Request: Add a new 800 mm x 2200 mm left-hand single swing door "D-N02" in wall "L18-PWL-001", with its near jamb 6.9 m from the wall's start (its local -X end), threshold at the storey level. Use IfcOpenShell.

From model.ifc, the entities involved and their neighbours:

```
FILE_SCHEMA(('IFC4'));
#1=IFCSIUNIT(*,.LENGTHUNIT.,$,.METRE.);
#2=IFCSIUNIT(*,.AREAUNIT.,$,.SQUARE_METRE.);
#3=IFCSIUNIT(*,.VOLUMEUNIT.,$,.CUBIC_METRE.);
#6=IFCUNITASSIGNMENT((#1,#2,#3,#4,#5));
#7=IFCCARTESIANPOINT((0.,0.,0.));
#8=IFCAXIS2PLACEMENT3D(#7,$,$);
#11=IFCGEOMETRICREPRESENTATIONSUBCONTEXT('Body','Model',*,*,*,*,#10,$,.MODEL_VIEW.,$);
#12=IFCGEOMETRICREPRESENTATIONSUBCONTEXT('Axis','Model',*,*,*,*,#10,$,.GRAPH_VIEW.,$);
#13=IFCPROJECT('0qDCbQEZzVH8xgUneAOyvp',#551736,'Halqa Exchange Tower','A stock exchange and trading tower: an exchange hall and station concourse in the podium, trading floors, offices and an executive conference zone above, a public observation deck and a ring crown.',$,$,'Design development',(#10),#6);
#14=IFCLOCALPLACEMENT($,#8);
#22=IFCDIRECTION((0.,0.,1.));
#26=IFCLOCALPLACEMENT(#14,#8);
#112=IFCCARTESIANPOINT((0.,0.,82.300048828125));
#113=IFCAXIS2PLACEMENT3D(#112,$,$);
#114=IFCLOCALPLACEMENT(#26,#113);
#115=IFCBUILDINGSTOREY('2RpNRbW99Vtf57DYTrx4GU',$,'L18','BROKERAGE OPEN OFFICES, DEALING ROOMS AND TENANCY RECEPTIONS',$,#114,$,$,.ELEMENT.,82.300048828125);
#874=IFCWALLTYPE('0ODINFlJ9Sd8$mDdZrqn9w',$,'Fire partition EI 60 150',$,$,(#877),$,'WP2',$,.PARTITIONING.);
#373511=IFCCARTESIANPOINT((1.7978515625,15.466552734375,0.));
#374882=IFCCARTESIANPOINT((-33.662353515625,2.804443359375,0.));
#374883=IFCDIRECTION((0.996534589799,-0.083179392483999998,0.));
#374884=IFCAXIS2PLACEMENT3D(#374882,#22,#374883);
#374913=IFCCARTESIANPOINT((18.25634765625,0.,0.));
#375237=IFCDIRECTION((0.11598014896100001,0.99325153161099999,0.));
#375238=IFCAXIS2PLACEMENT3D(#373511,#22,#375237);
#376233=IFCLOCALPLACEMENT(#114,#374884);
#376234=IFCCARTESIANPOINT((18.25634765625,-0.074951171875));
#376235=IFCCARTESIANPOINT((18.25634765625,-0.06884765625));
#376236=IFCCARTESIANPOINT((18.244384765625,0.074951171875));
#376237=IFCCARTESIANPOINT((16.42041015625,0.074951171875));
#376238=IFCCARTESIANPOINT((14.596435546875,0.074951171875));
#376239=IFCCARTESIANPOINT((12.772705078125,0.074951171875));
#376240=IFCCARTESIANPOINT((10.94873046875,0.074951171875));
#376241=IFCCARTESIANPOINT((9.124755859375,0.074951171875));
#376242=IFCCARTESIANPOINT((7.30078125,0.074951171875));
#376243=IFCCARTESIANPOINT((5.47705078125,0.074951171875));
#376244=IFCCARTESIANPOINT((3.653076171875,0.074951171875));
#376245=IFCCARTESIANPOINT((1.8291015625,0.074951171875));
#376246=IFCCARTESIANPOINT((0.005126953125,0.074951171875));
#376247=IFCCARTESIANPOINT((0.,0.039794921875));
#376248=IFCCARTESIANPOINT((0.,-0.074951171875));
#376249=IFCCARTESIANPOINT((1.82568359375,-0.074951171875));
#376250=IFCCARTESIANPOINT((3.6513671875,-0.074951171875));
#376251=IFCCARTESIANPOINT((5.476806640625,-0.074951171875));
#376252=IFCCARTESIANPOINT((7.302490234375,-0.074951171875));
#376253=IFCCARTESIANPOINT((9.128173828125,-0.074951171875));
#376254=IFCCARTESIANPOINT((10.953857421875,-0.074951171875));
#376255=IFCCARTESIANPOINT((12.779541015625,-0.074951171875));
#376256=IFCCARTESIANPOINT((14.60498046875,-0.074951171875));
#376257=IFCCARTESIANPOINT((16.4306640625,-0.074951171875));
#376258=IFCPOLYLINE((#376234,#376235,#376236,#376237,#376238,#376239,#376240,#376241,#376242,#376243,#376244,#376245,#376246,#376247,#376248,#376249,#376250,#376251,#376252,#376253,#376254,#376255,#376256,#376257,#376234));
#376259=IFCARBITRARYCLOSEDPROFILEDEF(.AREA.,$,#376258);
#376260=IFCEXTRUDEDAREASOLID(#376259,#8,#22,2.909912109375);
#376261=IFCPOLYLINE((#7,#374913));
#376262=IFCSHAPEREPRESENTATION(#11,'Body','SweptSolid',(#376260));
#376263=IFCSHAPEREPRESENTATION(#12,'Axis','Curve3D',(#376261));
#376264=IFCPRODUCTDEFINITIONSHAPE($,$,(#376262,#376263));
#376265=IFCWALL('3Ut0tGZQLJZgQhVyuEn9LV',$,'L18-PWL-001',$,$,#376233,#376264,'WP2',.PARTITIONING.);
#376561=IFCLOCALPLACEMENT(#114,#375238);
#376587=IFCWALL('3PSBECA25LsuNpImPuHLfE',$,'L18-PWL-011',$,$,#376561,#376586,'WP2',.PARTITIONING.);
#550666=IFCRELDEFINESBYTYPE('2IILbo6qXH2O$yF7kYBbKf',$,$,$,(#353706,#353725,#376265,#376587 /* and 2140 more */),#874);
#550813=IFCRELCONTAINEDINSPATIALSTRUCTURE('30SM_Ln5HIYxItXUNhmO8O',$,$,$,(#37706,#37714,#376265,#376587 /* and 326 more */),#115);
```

```python
import numpy as np
import ifcopenshell
import ifcopenshell.api.feature
import ifcopenshell.api.geometry
import ifcopenshell.api.root
import ifcopenshell.api.spatial
import ifcopenshell.geom
import ifcopenshell.util.element
import ifcopenshell.util.placement
import ifcopenshell.util.representation
import ifcopenshell.util.shape
import ifcopenshell.util.unit

model = ifcopenshell.open("model.ifc")
unit_scale = ifcopenshell.util.unit.calculate_unit_scale(model)
settings = ifcopenshell.geom.settings()


def volume(element):
    """Net volume in cubic metres, openings subtracted."""
    shape = ifcopenshell.geom.create_shape(settings, element)
    return ifcopenshell.util.shape.get_volume(shape.geometry)


wall = model.by_guid("3Ut0tGZQLJZgQhVyuEn9LV")
storey = ifcopenshell.util.element.get_container(wall, ifc_class="IfcBuildingStorey")
context = ifcopenshell.util.representation.get_context(model, "Model", "Body", "MODEL_VIEW")
before = volume(wall)

width, height, from_end, sill = 0.8, 2.2, 6.9, 0.0  # metres

# The wall runs along its own X axis, and the end named is its -X end.
wall_shape = ifcopenshell.geom.create_shape(settings, wall)
x, y, z = ifcopenshell.util.shape.get_vertices(wall_shape.geometry).T
start = x.min() + from_end
face, thickness = float(y.min()), float(y.max() - y.min())
wall_matrix = ifcopenshell.util.placement.get_local_placement(wall.ObjectPlacement)
level = ifcopenshell.util.placement.get_local_placement(storey.ObjectPlacement)[2, 3]


def in_wall(x, y):
    """Placement at x, y metres in the wall's axes, at sill height."""
    matrix = wall_matrix.copy()
    matrix[:, 3] = wall_matrix @ np.array([x / unit_scale, y / unit_scale, 0.0, 1.0])
    matrix[2, 3] = level + sill / unit_scale
    return matrix


# Opening: a box that overshoots both wall faces by 50 mm.
opening = ifcopenshell.api.root.create_entity(model, ifc_class="IfcOpeningElement", predefined_type="OPENING")
box = ifcopenshell.api.geometry.add_wall_representation(
    model, context=context, length=width, height=height, thickness=thickness + 0.1
)
ifcopenshell.api.geometry.assign_representation(model, product=opening, representation=box)
ifcopenshell.api.geometry.edit_object_placement(model, product=opening, matrix=in_wall(start, face - 0.05), is_si=False)
ifcopenshell.api.feature.add_feature(model, feature=opening, element=wall)

door = ifcopenshell.api.root.create_entity(model, ifc_class="IfcDoor", name="D-N02", predefined_type="DOOR")
door.OverallWidth, door.OverallHeight = width / unit_scale, height / unit_scale
door.OperationType = "SINGLE_SWING_LEFT"
body = ifcopenshell.api.geometry.add_door_representation(
    model,
    context=context,
    overall_width=door.OverallWidth,
    overall_height=door.OverallHeight,
    operation_type="SINGLE_SWING_LEFT",
    lining_properties={"LiningDepth": thickness / unit_scale, "ThresholdDepth": thickness / unit_scale},
)
ifcopenshell.api.geometry.assign_representation(model, product=door, representation=body)
ifcopenshell.api.spatial.assign_container(model, products=[door], relating_structure=storey)
ifcopenshell.api.feature.add_filling(model, opening=opening, element=door)

# The lining spans the wall, so the door starts at the wall face.
ifcopenshell.api.geometry.edit_object_placement(model, product=door, matrix=in_wall(start, face), is_si=False)

after = volume(wall)

print(f"wall volume {before:.3f} -> {after:.3f} m3")

model.write("model_rev.ifc")
```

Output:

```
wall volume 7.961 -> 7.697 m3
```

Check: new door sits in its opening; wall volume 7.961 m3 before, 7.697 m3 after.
